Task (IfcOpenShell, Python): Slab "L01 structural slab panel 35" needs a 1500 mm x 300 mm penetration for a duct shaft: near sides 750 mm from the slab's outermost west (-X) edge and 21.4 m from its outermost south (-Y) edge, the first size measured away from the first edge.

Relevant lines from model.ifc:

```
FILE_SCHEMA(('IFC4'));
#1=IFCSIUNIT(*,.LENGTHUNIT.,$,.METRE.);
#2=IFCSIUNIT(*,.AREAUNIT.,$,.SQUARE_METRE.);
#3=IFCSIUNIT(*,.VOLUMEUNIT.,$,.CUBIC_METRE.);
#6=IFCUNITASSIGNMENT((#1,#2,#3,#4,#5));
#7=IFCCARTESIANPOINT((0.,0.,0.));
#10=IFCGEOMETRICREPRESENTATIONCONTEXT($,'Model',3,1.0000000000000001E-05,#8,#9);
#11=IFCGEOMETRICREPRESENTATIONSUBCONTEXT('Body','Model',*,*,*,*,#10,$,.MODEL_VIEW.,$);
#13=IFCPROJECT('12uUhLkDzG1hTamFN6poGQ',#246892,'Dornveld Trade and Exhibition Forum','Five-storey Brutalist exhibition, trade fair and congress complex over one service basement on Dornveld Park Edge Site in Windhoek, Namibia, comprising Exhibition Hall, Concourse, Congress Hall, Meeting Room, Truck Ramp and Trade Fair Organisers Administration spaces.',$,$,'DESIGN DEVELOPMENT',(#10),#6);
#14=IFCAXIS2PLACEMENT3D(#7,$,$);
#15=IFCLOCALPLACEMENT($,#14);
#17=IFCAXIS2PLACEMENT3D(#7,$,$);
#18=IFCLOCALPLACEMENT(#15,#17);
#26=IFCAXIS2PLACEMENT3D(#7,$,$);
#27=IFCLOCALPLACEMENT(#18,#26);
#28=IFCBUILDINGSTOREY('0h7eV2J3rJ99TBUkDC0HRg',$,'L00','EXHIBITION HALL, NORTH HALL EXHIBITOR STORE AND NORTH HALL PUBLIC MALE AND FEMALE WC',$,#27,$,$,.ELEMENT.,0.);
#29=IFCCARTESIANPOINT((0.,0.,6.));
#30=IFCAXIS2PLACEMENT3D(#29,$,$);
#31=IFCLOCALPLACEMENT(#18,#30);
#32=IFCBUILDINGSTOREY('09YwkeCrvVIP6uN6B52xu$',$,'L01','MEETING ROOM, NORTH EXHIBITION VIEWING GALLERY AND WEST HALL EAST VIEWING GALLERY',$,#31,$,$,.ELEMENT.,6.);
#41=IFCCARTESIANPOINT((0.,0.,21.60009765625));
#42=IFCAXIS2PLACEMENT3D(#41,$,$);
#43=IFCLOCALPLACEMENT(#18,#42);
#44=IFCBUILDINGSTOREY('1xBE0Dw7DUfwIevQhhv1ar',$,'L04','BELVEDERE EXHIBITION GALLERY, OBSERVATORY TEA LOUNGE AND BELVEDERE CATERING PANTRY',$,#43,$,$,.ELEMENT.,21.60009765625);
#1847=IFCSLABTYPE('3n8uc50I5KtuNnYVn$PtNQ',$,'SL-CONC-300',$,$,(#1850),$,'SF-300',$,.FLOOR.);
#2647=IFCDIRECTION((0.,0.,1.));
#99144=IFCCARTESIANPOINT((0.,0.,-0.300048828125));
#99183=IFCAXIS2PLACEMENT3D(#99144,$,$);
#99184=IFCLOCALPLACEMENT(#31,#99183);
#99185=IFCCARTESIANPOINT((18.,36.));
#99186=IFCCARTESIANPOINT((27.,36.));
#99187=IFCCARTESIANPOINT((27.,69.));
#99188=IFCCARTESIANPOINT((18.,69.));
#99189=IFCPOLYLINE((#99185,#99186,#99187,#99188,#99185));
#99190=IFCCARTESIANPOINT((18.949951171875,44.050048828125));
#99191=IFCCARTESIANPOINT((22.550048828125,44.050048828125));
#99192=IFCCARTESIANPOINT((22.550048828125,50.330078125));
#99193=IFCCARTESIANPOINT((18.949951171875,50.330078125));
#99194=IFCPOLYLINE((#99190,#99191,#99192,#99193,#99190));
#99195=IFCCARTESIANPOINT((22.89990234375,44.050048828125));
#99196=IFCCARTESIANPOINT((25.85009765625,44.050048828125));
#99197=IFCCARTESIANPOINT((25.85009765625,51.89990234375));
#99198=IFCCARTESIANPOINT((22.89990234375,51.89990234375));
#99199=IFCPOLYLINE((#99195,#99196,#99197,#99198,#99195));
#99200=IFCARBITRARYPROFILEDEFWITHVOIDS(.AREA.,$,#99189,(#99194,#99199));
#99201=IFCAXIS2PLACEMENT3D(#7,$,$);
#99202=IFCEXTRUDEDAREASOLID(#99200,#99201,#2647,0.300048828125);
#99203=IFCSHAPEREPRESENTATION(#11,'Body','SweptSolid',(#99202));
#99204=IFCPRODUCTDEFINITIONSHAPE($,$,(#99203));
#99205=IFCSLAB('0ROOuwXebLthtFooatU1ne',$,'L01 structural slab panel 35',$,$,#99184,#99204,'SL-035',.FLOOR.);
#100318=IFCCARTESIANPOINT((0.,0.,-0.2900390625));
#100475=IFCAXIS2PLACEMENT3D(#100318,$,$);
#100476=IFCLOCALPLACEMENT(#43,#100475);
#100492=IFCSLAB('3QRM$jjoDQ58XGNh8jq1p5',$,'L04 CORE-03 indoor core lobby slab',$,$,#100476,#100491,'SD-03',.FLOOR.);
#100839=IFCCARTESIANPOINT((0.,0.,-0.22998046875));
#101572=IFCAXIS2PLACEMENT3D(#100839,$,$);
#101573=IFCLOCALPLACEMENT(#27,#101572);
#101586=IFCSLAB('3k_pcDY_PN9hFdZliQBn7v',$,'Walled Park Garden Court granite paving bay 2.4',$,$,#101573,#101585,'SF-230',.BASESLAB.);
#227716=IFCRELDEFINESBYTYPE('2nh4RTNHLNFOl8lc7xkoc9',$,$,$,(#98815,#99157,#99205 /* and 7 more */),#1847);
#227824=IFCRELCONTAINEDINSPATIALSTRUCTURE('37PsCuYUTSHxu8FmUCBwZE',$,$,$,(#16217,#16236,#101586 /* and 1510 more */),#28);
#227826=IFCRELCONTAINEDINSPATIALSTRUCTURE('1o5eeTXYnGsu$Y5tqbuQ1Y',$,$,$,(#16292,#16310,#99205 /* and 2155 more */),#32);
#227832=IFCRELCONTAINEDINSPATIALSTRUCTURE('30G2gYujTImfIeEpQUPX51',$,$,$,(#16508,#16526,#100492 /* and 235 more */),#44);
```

```python
import numpy as np
import ifcopenshell
import ifcopenshell.api.feature
import ifcopenshell.api.geometry
import ifcopenshell.api.root
import ifcopenshell.geom
import ifcopenshell.util.placement
import ifcopenshell.util.representation
import ifcopenshell.util.shape
import ifcopenshell.util.unit

model = ifcopenshell.open("model.ifc")
unit_scale = ifcopenshell.util.unit.calculate_unit_scale(model)
settings = ifcopenshell.geom.settings()


def volume(element):
    """Net volume in cubic metres, openings subtracted."""
    shape = ifcopenshell.geom.create_shape(settings, element)
    return ifcopenshell.util.shape.get_volume(shape.geometry)


slab = model.by_guid("0ROOuwXebLthtFooatU1ne")
before = volume(slab)

# Extent in the slab's own axes, in metres. The edges named are its -X and -Y sides.
slab_shape = ifcopenshell.geom.create_shape(settings, slab)
vertices = ifcopenshell.util.shape.get_vertices(slab_shape.geometry)
x_min, y_min, bottom = vertices.min(axis=0)
top = vertices[:, 2].max()

opening = ifcopenshell.api.root.create_entity(model, ifc_class="IfcOpeningElement", name="Duct shaft opening", predefined_type="OPENING")
context = ifcopenshell.util.representation.get_context(model, "Model", "Body", "MODEL_VIEW")
width, depth = 1.5, 0.3
outline = [(0.0, 0.0), (width, 0.0), (width, depth), (0.0, depth), (0.0, 0.0)]
# Overshoot both faces by 50 mm so the cut is clean.
shape = ifcopenshell.api.geometry.add_slab_representation(
    model, context=context, depth=top - bottom + 0.1, polyline=outline
)
ifcopenshell.api.geometry.assign_representation(model, product=opening, representation=shape)

matrix = ifcopenshell.util.placement.get_local_placement(slab.ObjectPlacement)
matrix[:, 3] = matrix @ np.append(np.array([x_min + 0.75, y_min + 21.4, bottom - 0.05]) / unit_scale, 1.0)
ifcopenshell.api.geometry.edit_object_placement(model, product=opening, matrix=matrix, is_si=False)
ifcopenshell.api.feature.add_feature(model, feature=opening, element=slab)

after = volume(slab)

print(f"slab volume {before:.3f} -> {after:.3f} m3")

model.write("model_updated.ifc")
```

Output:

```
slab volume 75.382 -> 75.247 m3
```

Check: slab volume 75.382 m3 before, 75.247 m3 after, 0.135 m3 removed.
